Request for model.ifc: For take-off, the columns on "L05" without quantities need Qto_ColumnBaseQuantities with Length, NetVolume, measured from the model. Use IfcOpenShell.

First a look at what the model holds.

```python
import ifcopenshell
import ifcopenshell.util.element
import ifcopenshell.util.unit

model = ifcopenshell.open("model.ifc")
print(model.schema)
for unit_type in ("LENGTHUNIT", "AREAUNIT", "VOLUMEUNIT"):
    print(unit_type, ifcopenshell.util.unit.calculate_unit_scale(model, unit_type))
storey = next(s for s in model.by_type("IfcBuildingStorey") if s.Name == "L05")
columns = [e for e in ifcopenshell.util.element.get_decomposition(storey) if e.is_a("IfcColumn")]
for e in sorted(columns, key=lambda e: e.id()):
    print(e.id(), e.is_a(), e.Name, list(ifcopenshell.util.element.get_psets(e, qtos_only=True)), sep=" | ")
```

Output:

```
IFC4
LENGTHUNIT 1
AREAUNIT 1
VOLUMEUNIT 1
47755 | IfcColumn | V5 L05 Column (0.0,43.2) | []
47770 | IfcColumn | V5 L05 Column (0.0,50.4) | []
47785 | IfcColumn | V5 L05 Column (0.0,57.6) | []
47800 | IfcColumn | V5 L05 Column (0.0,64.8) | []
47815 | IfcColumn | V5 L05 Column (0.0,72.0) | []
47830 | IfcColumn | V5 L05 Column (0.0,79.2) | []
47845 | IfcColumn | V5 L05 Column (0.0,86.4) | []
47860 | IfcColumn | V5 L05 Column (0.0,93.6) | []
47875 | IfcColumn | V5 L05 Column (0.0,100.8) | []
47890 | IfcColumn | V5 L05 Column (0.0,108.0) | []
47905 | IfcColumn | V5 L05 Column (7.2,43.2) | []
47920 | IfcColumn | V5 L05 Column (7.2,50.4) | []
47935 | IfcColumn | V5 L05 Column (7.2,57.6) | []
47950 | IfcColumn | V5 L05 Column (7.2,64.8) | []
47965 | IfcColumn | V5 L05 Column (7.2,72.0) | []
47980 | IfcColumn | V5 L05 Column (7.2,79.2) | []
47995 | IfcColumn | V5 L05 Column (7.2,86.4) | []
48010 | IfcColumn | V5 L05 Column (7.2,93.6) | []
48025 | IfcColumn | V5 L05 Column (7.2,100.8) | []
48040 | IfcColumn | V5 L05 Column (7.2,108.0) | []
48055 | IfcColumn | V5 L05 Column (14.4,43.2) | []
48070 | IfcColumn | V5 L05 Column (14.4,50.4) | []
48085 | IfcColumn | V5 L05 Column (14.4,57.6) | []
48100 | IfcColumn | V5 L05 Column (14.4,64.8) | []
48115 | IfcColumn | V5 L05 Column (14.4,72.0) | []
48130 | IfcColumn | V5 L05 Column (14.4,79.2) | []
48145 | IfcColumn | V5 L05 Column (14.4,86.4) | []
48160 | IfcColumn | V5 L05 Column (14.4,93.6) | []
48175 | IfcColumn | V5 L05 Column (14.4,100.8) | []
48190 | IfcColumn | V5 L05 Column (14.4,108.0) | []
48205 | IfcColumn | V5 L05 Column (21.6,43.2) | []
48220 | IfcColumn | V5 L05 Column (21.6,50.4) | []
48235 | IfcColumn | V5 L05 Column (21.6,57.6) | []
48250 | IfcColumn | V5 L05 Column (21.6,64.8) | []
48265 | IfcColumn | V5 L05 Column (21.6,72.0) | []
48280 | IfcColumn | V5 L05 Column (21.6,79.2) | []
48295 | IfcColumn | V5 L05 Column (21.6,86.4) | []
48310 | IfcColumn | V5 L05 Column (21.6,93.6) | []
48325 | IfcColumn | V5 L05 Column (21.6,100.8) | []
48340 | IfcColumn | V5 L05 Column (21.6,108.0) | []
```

```python
import ifcopenshell
import ifcopenshell.api.pset
import ifcopenshell.geom
import ifcopenshell.util.element
import ifcopenshell.util.shape
import ifcopenshell.util.unit

model = ifcopenshell.open("model.ifc")
unit_scale = ifcopenshell.util.unit.calculate_unit_scale(model)
volume_scale = ifcopenshell.util.unit.calculate_unit_scale(model, "VOLUMEUNIT")
settings = ifcopenshell.geom.settings()

storey = next(s for s in model.by_type("IfcBuildingStorey") if s.Name == "L05")
columns = [e for e in ifcopenshell.util.element.get_decomposition(storey) if e.is_a("IfcColumn")]

for e in sorted(columns, key=lambda e: e.id()):
    if ifcopenshell.util.element.get_psets(e, qtos_only=True, should_inherit=False):
        continue
    # Geometry comes back in metres, in the element's own axes.
    shape = ifcopenshell.geom.create_shape(settings, e)
    values = {
        "Length": ifcopenshell.util.shape.get_z(shape.geometry) / unit_scale,
        "NetVolume": ifcopenshell.util.shape.get_volume(shape.geometry) / volume_scale,
    }
    qto = ifcopenshell.api.pset.add_qto(model, product=e, name="Qto_ColumnBaseQuantities")
    ifcopenshell.api.pset.edit_qto(model, qto=qto, properties=values)
    print(e.id(), {k: round(v, 3) for k, v in values.items()})

model.write("model_updated.ifc")
```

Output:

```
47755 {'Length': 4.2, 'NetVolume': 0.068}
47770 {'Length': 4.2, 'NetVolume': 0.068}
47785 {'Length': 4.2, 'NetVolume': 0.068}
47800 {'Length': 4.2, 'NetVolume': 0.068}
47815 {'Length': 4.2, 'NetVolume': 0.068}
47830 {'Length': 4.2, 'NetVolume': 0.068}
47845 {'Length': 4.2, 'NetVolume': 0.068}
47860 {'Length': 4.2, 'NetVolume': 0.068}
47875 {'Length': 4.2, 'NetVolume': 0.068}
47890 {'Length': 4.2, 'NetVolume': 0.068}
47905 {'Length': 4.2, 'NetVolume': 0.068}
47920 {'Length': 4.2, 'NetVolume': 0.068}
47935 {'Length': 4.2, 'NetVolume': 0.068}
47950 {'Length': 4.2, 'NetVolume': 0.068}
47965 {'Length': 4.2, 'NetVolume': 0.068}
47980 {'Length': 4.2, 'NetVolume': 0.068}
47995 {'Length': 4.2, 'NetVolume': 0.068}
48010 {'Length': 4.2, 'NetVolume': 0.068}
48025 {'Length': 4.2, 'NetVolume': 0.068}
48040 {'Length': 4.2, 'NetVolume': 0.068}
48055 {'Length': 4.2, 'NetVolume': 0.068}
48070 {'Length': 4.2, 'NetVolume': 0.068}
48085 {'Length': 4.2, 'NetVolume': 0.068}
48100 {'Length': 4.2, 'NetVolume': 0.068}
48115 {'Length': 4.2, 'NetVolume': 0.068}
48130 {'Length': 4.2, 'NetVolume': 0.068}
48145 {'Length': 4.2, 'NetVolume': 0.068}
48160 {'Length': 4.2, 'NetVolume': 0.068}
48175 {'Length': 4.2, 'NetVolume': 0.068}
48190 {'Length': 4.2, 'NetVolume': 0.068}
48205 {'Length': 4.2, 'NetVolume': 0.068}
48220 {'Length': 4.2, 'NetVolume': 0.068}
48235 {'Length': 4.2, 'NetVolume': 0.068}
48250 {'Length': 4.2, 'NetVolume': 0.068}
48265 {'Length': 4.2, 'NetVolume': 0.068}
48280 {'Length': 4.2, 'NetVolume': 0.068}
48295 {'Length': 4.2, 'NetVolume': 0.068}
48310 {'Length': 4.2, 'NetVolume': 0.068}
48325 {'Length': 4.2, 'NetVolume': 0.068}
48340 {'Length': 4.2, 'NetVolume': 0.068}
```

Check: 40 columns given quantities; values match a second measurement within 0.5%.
